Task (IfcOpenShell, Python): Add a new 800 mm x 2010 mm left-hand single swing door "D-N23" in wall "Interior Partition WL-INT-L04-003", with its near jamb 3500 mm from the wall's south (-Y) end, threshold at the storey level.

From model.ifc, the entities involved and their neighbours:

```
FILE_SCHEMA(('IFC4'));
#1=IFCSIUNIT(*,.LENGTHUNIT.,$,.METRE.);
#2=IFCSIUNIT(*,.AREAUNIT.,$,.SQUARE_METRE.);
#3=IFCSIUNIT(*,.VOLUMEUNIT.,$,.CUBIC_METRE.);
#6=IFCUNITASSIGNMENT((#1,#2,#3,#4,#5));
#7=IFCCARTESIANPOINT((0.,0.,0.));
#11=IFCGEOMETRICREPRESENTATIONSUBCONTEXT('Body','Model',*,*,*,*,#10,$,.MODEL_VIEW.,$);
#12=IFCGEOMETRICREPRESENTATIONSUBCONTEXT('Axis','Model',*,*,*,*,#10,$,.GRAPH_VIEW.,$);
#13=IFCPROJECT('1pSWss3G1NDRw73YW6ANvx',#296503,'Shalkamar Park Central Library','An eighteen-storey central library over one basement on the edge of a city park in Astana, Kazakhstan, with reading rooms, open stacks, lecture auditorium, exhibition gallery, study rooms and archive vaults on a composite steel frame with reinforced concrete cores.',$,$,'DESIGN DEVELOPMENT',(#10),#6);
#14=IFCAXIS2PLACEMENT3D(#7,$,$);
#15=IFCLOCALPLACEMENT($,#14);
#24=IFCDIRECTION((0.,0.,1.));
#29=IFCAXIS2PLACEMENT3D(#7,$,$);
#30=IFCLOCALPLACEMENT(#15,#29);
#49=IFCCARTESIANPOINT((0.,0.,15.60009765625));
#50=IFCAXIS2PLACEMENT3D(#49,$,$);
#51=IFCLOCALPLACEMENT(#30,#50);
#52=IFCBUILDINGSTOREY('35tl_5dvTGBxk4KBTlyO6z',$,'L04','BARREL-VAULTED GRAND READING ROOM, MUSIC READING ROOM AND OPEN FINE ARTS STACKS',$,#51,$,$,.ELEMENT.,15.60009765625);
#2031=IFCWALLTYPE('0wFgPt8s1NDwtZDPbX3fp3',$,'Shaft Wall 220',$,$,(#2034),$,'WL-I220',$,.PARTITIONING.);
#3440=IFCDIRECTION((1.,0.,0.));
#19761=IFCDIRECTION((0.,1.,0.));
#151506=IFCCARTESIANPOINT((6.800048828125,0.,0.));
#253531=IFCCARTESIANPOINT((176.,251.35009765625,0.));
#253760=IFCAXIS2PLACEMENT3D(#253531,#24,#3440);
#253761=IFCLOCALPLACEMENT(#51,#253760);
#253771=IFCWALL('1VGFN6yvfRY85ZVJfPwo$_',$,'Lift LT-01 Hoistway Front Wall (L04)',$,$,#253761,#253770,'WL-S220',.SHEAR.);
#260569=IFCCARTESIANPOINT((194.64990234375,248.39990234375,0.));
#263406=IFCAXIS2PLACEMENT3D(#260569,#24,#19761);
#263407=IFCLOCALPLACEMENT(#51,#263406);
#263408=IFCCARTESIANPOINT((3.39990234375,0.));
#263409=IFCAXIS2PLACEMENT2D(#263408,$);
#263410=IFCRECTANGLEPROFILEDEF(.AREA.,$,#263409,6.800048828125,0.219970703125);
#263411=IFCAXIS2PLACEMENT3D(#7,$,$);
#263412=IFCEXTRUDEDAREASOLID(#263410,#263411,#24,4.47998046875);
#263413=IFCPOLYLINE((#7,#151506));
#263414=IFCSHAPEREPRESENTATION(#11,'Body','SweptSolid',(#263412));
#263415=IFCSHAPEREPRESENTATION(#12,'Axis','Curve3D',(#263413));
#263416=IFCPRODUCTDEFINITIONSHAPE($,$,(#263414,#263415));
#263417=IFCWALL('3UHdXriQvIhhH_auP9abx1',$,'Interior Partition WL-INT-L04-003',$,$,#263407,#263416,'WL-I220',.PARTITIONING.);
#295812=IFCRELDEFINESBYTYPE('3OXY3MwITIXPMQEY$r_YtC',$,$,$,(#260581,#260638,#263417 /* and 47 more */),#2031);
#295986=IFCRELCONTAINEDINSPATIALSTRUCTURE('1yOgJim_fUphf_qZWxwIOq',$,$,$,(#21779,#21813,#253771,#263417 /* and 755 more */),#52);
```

```python
import numpy as np
import ifcopenshell
import ifcopenshell.api.feature
import ifcopenshell.api.geometry
import ifcopenshell.api.root
import ifcopenshell.api.spatial
import ifcopenshell.geom
import ifcopenshell.util.element
import ifcopenshell.util.placement
import ifcopenshell.util.representation
import ifcopenshell.util.shape
import ifcopenshell.util.unit

model = ifcopenshell.open("model.ifc")
unit_scale = ifcopenshell.util.unit.calculate_unit_scale(model)
settings = ifcopenshell.geom.settings()


def volume(element):
    """Net volume in cubic metres, openings subtracted."""
    shape = ifcopenshell.geom.create_shape(settings, element)
    return ifcopenshell.util.shape.get_volume(shape.geometry)


wall = model.by_guid("3UHdXriQvIhhH_auP9abx1")
storey = ifcopenshell.util.element.get_container(wall, ifc_class="IfcBuildingStorey")
context = ifcopenshell.util.representation.get_context(model, "Model", "Body", "MODEL_VIEW")
before = volume(wall)

width, height, from_end, sill = 0.8, 2.01, 3.5, 0.0  # metres

# The wall runs along its own X axis, and the end named is its -X end.
wall_shape = ifcopenshell.geom.create_shape(settings, wall)
x, y, z = ifcopenshell.util.shape.get_vertices(wall_shape.geometry).T
start = x.min() + from_end
face, thickness = float(y.min()), float(y.max() - y.min())
wall_matrix = ifcopenshell.util.placement.get_local_placement(wall.ObjectPlacement)
level = ifcopenshell.util.placement.get_local_placement(storey.ObjectPlacement)[2, 3]


def in_wall(x, y):
    """Placement at x, y metres in the wall's axes, at sill height."""
    matrix = wall_matrix.copy()
    matrix[:, 3] = wall_matrix @ np.array([x / unit_scale, y / unit_scale, 0.0, 1.0])
    matrix[2, 3] = level + sill / unit_scale
    return matrix


# Opening: a box that overshoots both wall faces by 50 mm.
opening = ifcopenshell.api.root.create_entity(model, ifc_class="IfcOpeningElement", predefined_type="OPENING")
box = ifcopenshell.api.geometry.add_wall_representation(
    model, context=context, length=width, height=height, thickness=thickness + 0.1
)
ifcopenshell.api.geometry.assign_representation(model, product=opening, representation=box)
ifcopenshell.api.geometry.edit_object_placement(model, product=opening, matrix=in_wall(start, face - 0.05), is_si=False)
ifcopenshell.api.feature.add_feature(model, feature=opening, element=wall)

door = ifcopenshell.api.root.create_entity(model, ifc_class="IfcDoor", name="D-N23", predefined_type="DOOR")
door.OverallWidth, door.OverallHeight = width / unit_scale, height / unit_scale
door.OperationType = "SINGLE_SWING_LEFT"
body = ifcopenshell.api.geometry.add_door_representation(
    model,
    context=context,
    overall_width=door.OverallWidth,
    overall_height=door.OverallHeight,
    operation_type="SINGLE_SWING_LEFT",
    lining_properties={"LiningDepth": thickness / unit_scale, "ThresholdDepth": thickness / unit_scale},
)
ifcopenshell.api.geometry.assign_representation(model, product=door, representation=body)
ifcopenshell.api.spatial.assign_container(model, products=[door], relating_structure=storey)
ifcopenshell.api.feature.add_filling(model, opening=opening, element=door)

# The lining spans the wall, so the door starts at the wall face.
ifcopenshell.api.geometry.edit_object_placement(model, product=door, matrix=in_wall(start, face), is_si=False)

after = volume(wall)

print(f"wall volume {before:.3f} -> {after:.3f} m3")

model.write("model_edited.ifc")
```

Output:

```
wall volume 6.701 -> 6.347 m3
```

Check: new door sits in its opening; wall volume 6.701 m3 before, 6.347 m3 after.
